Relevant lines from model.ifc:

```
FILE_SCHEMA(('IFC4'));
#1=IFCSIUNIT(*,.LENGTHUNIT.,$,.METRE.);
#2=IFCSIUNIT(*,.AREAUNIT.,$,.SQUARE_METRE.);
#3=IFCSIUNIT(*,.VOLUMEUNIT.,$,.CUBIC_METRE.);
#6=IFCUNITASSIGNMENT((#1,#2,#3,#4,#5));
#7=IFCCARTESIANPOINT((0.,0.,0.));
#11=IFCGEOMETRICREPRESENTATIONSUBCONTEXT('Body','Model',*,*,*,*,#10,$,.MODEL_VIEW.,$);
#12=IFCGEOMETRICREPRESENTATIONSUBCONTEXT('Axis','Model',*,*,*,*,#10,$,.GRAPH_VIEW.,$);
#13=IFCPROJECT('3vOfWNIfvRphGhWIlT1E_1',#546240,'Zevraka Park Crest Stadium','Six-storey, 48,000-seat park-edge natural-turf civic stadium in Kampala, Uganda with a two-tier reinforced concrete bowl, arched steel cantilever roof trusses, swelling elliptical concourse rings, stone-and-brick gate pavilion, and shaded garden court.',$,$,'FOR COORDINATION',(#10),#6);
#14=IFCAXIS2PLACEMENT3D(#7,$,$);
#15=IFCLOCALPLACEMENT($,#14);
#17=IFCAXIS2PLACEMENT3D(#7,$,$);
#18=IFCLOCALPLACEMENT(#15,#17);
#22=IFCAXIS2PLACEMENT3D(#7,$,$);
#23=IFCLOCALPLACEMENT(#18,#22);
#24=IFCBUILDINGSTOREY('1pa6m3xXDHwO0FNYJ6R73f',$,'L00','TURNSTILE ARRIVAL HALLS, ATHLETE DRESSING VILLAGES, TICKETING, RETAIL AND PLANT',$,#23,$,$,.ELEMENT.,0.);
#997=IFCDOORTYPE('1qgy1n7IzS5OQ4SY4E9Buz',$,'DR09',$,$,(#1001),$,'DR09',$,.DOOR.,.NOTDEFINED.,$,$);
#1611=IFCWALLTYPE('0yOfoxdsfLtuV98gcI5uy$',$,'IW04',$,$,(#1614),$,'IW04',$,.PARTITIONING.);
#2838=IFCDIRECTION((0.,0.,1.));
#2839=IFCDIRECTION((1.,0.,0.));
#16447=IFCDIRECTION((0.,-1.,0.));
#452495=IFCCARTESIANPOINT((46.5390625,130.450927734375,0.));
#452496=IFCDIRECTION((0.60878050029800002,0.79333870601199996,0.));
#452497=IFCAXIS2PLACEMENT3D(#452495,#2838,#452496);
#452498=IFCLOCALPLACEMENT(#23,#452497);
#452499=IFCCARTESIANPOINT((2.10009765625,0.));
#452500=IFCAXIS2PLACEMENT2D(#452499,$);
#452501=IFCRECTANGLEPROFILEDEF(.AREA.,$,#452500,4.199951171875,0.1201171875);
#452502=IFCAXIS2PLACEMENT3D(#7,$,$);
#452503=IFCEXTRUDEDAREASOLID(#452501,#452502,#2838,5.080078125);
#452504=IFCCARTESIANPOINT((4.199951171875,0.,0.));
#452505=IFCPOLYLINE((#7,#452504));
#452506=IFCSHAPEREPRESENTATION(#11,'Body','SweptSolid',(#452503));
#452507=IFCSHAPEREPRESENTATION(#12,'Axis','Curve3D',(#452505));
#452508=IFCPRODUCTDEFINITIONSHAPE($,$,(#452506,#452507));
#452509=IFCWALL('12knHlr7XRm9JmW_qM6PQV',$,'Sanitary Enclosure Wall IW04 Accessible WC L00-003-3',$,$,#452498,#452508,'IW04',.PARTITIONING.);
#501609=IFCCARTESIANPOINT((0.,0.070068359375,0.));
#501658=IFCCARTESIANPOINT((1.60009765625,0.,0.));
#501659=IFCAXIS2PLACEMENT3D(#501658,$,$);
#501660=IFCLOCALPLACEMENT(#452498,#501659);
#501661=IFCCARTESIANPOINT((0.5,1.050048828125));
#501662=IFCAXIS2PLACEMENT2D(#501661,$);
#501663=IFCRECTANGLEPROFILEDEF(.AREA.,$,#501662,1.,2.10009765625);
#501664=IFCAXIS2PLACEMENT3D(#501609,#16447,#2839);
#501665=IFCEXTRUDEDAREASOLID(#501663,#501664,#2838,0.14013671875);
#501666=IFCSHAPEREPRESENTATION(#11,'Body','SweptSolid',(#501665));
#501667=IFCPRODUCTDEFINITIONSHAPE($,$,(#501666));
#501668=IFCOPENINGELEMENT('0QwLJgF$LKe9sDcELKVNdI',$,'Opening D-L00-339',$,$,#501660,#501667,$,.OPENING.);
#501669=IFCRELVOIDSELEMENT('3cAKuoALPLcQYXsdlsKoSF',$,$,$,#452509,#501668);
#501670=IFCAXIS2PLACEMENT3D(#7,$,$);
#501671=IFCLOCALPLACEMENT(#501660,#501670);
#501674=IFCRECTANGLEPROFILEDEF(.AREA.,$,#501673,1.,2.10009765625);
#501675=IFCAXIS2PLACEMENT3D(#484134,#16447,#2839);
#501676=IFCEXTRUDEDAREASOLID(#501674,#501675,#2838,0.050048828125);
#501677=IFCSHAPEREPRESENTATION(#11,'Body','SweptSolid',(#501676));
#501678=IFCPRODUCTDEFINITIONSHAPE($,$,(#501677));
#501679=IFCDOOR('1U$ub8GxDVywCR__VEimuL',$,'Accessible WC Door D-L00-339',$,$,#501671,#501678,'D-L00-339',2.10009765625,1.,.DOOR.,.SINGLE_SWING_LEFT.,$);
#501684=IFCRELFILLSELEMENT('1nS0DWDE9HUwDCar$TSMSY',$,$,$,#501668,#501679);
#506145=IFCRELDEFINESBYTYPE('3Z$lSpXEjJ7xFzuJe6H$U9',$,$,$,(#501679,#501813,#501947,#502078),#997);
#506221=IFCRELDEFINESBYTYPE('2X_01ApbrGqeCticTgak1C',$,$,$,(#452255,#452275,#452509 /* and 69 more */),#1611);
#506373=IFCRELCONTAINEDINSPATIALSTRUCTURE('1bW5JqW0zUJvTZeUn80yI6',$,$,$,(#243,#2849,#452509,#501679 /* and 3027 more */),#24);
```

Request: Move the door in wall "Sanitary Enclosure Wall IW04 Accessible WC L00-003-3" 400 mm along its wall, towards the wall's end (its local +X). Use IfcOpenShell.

```python
import ifcopenshell
import ifcopenshell.api.geometry
import ifcopenshell.util.placement

model = ifcopenshell.open("model.ifc")

door = model.by_guid("1U$ub8GxDVywCR__VEimuL")
opening = door.FillsVoids[0].RelatingOpeningElement
wall = opening.VoidsElements[0].RelatingBuildingElement

wall_matrix = ifcopenshell.util.placement.get_local_placement(wall.ObjectPlacement)
shift = wall_matrix[:3, 0] * 0.4
before = ifcopenshell.util.placement.get_local_placement(door.ObjectPlacement)[:3, 3].copy()

# The door is placed relative to its opening, so it follows when the opening moves.
matrix = ifcopenshell.util.placement.get_local_placement(opening.ObjectPlacement)
matrix[:3, 3] += shift
ifcopenshell.api.geometry.edit_object_placement(
    model, product=opening, matrix=matrix, is_si=False, should_transform_children=True
)

after = ifcopenshell.util.placement.get_local_placement(door.ObjectPlacement)[:3, 3]
print("door moved by", (after - before).round(3) + 0.0)

model.write("model_edited.ifc")
```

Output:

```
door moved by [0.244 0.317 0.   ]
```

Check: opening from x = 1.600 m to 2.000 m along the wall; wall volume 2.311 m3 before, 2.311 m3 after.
